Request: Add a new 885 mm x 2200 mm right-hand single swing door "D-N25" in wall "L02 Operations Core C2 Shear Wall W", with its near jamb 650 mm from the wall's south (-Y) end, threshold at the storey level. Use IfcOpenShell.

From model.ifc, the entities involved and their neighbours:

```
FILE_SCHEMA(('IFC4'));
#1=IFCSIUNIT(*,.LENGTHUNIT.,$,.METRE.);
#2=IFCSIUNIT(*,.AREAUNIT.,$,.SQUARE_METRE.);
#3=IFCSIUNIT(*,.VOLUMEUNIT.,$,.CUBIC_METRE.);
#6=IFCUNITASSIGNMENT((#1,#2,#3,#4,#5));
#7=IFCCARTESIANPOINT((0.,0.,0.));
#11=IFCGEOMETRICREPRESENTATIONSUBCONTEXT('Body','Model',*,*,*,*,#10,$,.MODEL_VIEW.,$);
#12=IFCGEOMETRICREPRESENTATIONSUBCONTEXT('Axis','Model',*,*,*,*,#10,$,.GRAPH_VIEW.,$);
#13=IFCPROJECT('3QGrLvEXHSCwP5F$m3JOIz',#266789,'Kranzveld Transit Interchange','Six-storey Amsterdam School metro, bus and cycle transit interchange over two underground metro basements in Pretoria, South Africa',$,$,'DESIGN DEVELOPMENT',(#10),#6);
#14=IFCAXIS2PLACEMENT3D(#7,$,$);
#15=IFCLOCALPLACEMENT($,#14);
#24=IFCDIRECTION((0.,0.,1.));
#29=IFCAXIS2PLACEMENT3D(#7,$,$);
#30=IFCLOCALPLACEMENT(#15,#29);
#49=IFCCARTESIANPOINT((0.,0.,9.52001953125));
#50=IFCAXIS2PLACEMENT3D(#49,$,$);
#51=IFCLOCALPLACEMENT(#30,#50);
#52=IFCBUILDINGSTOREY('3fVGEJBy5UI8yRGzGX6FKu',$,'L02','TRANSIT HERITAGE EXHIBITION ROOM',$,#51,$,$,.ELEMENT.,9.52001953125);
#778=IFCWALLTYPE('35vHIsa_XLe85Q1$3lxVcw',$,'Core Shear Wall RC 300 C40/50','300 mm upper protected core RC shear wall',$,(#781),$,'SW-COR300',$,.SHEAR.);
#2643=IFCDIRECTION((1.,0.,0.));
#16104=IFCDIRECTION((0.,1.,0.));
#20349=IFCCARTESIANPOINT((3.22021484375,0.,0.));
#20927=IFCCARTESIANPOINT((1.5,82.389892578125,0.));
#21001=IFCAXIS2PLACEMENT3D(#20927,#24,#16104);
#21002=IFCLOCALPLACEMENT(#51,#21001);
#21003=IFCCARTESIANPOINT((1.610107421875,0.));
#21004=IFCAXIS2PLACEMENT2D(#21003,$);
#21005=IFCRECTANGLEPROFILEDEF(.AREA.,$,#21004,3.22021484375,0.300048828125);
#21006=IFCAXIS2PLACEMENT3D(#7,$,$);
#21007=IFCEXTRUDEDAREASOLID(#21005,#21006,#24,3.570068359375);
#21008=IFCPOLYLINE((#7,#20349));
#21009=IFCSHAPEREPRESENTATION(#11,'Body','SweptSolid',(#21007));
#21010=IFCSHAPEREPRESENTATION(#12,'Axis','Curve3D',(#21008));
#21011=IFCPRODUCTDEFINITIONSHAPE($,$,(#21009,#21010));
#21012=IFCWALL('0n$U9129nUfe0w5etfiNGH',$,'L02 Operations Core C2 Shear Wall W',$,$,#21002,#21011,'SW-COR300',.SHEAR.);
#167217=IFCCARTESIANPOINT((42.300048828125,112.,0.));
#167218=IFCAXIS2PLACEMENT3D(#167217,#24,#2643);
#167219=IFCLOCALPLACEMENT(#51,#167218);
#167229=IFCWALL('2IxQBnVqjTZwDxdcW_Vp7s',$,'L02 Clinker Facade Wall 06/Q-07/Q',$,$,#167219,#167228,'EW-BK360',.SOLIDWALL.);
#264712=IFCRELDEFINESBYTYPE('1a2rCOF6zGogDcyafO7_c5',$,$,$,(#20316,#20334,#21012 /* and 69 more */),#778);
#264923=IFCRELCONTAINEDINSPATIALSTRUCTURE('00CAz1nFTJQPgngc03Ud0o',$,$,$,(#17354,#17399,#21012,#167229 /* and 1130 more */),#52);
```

```python
import numpy as np
import ifcopenshell
import ifcopenshell.api.feature
import ifcopenshell.api.geometry
import ifcopenshell.api.root
import ifcopenshell.api.spatial
import ifcopenshell.geom
import ifcopenshell.util.element
import ifcopenshell.util.placement
import ifcopenshell.util.representation
import ifcopenshell.util.shape
import ifcopenshell.util.unit

model = ifcopenshell.open("model.ifc")
unit_scale = ifcopenshell.util.unit.calculate_unit_scale(model)
settings = ifcopenshell.geom.settings()


def volume(element):
    """Net volume in cubic metres, openings subtracted."""
    shape = ifcopenshell.geom.create_shape(settings, element)
    return ifcopenshell.util.shape.get_volume(shape.geometry)


wall = model.by_guid("0n$U9129nUfe0w5etfiNGH")
storey = ifcopenshell.util.element.get_container(wall, ifc_class="IfcBuildingStorey")
context = ifcopenshell.util.representation.get_context(model, "Model", "Body", "MODEL_VIEW")
before = volume(wall)

width, height, from_end, sill = 0.885, 2.2, 0.65, 0.0  # metres

# The wall runs along its own X axis, and the end named is its -X end.
wall_shape = ifcopenshell.geom.create_shape(settings, wall)
x, y, z = ifcopenshell.util.shape.get_vertices(wall_shape.geometry).T
start = x.min() + from_end
face, thickness = float(y.min()), float(y.max() - y.min())
wall_matrix = ifcopenshell.util.placement.get_local_placement(wall.ObjectPlacement)
level = ifcopenshell.util.placement.get_local_placement(storey.ObjectPlacement)[2, 3]


def in_wall(x, y):
    """Placement at x, y metres in the wall's axes, at sill height."""
    matrix = wall_matrix.copy()
    matrix[:, 3] = wall_matrix @ np.array([x / unit_scale, y / unit_scale, 0.0, 1.0])
    matrix[2, 3] = level + sill / unit_scale
    return matrix


# Opening: a box that overshoots both wall faces by 50 mm.
opening = ifcopenshell.api.root.create_entity(model, ifc_class="IfcOpeningElement", predefined_type="OPENING")
box = ifcopenshell.api.geometry.add_wall_representation(
    model, context=context, length=width, height=height, thickness=thickness + 0.1
)
ifcopenshell.api.geometry.assign_representation(model, product=opening, representation=box)
ifcopenshell.api.geometry.edit_object_placement(model, product=opening, matrix=in_wall(start, face - 0.05), is_si=False)
ifcopenshell.api.feature.add_feature(model, feature=opening, element=wall)

door = ifcopenshell.api.root.create_entity(model, ifc_class="IfcDoor", name="D-N25", predefined_type="DOOR")
door.OverallWidth, door.OverallHeight = width / unit_scale, height / unit_scale
door.OperationType = "SINGLE_SWING_RIGHT"
body = ifcopenshell.api.geometry.add_door_representation(
    model,
    context=context,
    overall_width=door.OverallWidth,
    overall_height=door.OverallHeight,
    operation_type="SINGLE_SWING_RIGHT",
    lining_properties={"LiningDepth": thickness / unit_scale, "ThresholdDepth": thickness / unit_scale},
)
ifcopenshell.api.geometry.assign_representation(model, product=door, representation=body)
ifcopenshell.api.spatial.assign_container(model, products=[door], relating_structure=storey)
ifcopenshell.api.feature.add_filling(model, opening=opening, element=door)

# The lining spans the wall, so the door starts at the wall face.
ifcopenshell.api.geometry.edit_object_placement(model, product=door, matrix=in_wall(start, face), is_si=False)

after = volume(wall)

print(f"wall volume {before:.3f} -> {after:.3f} m3")

model.write("model_edited.ifc")
```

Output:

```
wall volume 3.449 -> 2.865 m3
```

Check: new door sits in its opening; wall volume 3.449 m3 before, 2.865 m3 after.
